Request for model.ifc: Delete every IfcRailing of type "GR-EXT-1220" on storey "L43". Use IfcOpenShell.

First a look at what the model holds.

```python
import ifcopenshell
import ifcopenshell.util.element

model = ifcopenshell.open("model.ifc")
print(model.schema)
storey = next(s for s in model.by_type("IfcBuildingStorey") if s.Name == "L43")
railings = [e for e in ifcopenshell.util.element.get_decomposition(storey) if e.is_a("IfcRailing")]
seen = {}
for e in railings:
    element_type = ifcopenshell.util.element.get_type(e)
    name = element_type.Name if element_type not in (None, e) else None
    seen[name] = seen.get(name, 0) + 1
for name, count in sorted(seen.items(), key=str):
    print(count, "x", name)
```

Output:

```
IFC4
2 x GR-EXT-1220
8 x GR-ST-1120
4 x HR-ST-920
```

```python
import ifcopenshell
import ifcopenshell.api.root
import ifcopenshell.util.element

model = ifcopenshell.open("model.ifc")

storey = next(s for s in model.by_type("IfcBuildingStorey") if s.Name == "L43")
railings = [e for e in ifcopenshell.util.element.get_decomposition(storey) if e.is_a("IfcRailing")]
targets = [e for e in railings if (t := ifcopenshell.util.element.get_type(e)) not in (None, e) and t.Name == "GR-EXT-1220"]

for e in targets:
    ifcopenshell.api.root.remove_product(model, product=e)
print(len(targets), "removed")

model.write("model_updated.ifc")
```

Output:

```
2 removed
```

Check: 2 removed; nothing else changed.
